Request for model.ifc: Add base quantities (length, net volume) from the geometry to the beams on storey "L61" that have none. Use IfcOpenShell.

First a look at what the model holds.

```python
import ifcopenshell
import ifcopenshell.util.element
import ifcopenshell.util.unit

model = ifcopenshell.open("model.ifc")
print(model.schema)
for unit_type in ("LENGTHUNIT", "AREAUNIT", "VOLUMEUNIT"):
    print(unit_type, ifcopenshell.util.unit.calculate_unit_scale(model, unit_type))
storey = next(s for s in model.by_type("IfcBuildingStorey") if s.Name == "L61")
beams = [e for e in ifcopenshell.util.element.get_decomposition(storey) if e.is_a("IfcBeam")]
for e in sorted(beams, key=lambda e: e.id()):
    print(e.id(), e.is_a(), e.Name, list(ifcopenshell.util.element.get_psets(e, qtos_only=True)), sep=" | ")
```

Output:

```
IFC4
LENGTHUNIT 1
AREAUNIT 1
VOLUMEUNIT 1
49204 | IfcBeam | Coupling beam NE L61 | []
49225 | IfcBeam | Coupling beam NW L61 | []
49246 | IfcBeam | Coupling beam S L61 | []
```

```python
import ifcopenshell
import ifcopenshell.api.pset
import ifcopenshell.geom
import ifcopenshell.util.element
import ifcopenshell.util.shape
import ifcopenshell.util.unit

model = ifcopenshell.open("model.ifc")
unit_scale = ifcopenshell.util.unit.calculate_unit_scale(model)
volume_scale = ifcopenshell.util.unit.calculate_unit_scale(model, "VOLUMEUNIT")
settings = ifcopenshell.geom.settings()

storey = next(s for s in model.by_type("IfcBuildingStorey") if s.Name == "L61")
beams = [e for e in ifcopenshell.util.element.get_decomposition(storey) if e.is_a("IfcBeam")]

for e in sorted(beams, key=lambda e: e.id()):
    if ifcopenshell.util.element.get_psets(e, qtos_only=True, should_inherit=False):
        continue
    # Geometry comes back in metres, in the element's own axes.
    shape = ifcopenshell.geom.create_shape(settings, e)
    values = {
        "Length": ifcopenshell.util.shape.get_max_xyz(shape.geometry) / unit_scale,
        "NetVolume": ifcopenshell.util.shape.get_volume(shape.geometry) / volume_scale,
    }
    qto = ifcopenshell.api.pset.add_qto(model, product=e, name="Qto_BeamBaseQuantities")
    ifcopenshell.api.pset.edit_qto(model, qto=qto, properties=values)
    print(e.id(), {k: round(v, 3) for k, v in values.items()})

model.write("model_edited.ifc")
```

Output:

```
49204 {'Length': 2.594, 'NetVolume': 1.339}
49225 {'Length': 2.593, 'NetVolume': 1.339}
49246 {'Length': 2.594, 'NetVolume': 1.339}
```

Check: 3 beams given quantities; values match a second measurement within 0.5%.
